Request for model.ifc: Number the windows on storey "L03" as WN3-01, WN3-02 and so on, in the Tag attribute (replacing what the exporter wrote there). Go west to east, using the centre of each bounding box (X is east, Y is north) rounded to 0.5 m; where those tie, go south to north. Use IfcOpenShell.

First a look at what the model holds.

```python
import ifcopenshell
import ifcopenshell.util.element
import ifcopenshell.util.placement

model = ifcopenshell.open("model.ifc")
print(model.schema)
storey = next(s for s in model.by_type("IfcBuildingStorey") if s.Name == "L03")
windows = [e for e in ifcopenshell.util.element.get_decomposition(storey) if e.is_a("IfcWindow")]
for e in sorted(windows, key=lambda e: e.id()):
    origin = ifcopenshell.util.placement.get_local_placement(e.ObjectPlacement)[:3, 3]
    print(e.id(), e.Tag, e.Name, origin.round(2) + 0.0, sep=" | ")
```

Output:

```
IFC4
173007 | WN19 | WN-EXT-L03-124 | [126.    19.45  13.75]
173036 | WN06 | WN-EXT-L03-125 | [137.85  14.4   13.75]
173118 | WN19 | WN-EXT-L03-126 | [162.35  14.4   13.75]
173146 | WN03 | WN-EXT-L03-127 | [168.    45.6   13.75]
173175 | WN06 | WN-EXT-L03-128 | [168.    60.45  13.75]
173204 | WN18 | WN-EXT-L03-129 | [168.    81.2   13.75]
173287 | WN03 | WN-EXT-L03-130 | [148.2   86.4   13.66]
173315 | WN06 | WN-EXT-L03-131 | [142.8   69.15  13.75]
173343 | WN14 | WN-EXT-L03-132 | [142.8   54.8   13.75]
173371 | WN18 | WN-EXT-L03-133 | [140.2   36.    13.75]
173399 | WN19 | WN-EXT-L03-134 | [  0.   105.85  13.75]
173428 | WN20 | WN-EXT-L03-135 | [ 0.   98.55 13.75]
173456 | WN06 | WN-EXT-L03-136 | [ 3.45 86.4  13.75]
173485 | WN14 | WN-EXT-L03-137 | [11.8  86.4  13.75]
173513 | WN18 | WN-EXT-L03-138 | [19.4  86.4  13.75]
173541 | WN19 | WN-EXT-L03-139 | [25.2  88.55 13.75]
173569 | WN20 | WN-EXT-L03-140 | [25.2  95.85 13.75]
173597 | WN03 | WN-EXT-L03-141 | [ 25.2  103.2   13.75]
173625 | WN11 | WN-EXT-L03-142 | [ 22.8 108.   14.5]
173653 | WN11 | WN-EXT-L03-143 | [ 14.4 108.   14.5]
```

```python
import ifcopenshell
import ifcopenshell.geom
import ifcopenshell.util.element
import ifcopenshell.util.shape

model = ifcopenshell.open("model.ifc")
settings = ifcopenshell.geom.settings()
settings.set("use-world-coords", True)


def centre(element):
    shape = ifcopenshell.geom.create_shape(settings, element)
    return ifcopenshell.util.shape.get_bbox_centroid(shape.geometry)


storey = next(s for s in model.by_type("IfcBuildingStorey") if s.Name == "L03")
windows = [e for e in ifcopenshell.util.element.get_decomposition(storey) if e.is_a("IfcWindow")]

# Insertion points can sit at a corner or the storey origin, so sort by the geometry (in metres).
centres = {e: centre(e) for e in windows}
windows.sort(key=lambda e: (round(centres[e][0] / 0.5), centres[e][1]))

for i, e in enumerate(windows, start=1):
    number = f"WN3-{i:02d}"
    e.Tag = number
    print(e.id(), number)

model.write("model_edited.ifc")
```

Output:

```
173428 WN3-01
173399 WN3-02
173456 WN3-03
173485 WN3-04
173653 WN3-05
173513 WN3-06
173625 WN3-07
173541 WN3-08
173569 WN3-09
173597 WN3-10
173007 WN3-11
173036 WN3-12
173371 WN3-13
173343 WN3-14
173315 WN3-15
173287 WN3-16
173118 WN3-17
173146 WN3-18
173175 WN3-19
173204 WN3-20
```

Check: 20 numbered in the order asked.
